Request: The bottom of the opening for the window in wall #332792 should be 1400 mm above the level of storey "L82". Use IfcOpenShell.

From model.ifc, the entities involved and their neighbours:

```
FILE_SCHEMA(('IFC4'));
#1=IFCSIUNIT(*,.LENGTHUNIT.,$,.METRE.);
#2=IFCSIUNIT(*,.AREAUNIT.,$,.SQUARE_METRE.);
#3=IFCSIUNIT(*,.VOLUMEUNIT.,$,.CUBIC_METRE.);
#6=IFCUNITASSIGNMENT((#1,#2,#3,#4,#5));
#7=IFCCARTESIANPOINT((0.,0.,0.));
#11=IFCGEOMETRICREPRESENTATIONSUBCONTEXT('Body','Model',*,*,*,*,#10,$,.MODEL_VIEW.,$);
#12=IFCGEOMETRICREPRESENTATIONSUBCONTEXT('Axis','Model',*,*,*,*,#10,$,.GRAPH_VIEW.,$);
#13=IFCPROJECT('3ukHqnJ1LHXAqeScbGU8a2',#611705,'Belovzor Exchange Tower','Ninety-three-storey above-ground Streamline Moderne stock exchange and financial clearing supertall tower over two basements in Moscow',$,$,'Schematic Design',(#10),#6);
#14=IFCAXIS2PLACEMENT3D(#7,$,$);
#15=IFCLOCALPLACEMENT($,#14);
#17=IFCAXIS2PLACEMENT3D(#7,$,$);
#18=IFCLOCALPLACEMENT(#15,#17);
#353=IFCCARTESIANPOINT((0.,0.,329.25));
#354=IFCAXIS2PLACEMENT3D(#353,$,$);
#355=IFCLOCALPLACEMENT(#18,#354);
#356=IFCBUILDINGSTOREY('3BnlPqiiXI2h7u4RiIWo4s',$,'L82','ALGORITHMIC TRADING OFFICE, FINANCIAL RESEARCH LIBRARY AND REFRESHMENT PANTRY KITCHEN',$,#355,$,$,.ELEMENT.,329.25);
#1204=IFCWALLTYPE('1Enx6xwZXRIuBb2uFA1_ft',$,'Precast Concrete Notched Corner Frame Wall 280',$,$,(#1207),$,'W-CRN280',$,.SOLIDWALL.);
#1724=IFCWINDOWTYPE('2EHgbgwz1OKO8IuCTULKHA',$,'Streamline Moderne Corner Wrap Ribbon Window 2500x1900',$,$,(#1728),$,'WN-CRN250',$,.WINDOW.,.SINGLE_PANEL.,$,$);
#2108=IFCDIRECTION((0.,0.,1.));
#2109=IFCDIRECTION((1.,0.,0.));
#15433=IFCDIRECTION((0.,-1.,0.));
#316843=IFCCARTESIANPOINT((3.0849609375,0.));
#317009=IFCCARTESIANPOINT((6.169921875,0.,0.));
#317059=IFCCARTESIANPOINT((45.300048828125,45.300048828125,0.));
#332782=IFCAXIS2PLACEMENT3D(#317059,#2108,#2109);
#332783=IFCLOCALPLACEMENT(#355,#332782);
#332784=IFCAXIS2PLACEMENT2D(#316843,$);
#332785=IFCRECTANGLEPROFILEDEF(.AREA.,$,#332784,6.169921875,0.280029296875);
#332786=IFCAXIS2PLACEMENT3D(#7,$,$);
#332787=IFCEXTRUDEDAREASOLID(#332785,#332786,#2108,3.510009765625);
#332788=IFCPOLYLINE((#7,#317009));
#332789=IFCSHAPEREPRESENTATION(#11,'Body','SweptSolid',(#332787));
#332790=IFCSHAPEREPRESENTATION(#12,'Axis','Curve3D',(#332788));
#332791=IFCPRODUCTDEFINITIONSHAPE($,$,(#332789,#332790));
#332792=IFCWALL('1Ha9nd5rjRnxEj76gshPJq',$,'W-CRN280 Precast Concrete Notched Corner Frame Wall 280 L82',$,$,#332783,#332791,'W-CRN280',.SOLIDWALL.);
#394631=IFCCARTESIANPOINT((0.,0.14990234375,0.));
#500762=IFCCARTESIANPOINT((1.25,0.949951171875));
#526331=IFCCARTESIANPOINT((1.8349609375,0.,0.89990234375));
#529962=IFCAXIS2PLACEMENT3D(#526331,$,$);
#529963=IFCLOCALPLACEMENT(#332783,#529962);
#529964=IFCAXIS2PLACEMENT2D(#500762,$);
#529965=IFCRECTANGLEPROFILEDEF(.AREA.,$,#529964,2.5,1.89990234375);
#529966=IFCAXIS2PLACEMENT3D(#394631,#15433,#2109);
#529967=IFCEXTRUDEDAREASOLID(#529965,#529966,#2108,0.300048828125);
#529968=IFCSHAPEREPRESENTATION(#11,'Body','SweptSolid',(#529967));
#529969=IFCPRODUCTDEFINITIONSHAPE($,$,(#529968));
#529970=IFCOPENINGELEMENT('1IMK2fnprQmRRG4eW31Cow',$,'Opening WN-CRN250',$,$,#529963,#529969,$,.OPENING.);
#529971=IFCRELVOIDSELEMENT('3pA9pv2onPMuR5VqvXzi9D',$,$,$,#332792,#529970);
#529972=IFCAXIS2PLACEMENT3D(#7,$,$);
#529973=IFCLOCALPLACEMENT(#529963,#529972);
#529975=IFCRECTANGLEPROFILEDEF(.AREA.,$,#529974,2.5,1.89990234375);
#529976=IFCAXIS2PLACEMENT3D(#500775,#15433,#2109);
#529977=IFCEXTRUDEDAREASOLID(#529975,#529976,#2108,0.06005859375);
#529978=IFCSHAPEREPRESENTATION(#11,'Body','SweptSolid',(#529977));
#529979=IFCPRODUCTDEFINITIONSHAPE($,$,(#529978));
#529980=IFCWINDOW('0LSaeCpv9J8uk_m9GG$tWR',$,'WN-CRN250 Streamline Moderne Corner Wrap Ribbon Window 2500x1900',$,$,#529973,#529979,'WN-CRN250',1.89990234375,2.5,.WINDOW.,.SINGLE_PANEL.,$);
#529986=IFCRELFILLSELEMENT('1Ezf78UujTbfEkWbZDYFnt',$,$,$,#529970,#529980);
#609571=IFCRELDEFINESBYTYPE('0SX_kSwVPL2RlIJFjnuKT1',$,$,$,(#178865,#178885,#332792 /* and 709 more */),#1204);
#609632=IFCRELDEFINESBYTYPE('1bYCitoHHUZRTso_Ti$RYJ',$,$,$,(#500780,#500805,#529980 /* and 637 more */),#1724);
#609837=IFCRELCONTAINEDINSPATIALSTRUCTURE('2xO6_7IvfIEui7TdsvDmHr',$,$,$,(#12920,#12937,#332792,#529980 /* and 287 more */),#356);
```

```python
import numpy as np
import ifcopenshell
import ifcopenshell.api.geometry
import ifcopenshell.geom
import ifcopenshell.util.element
import ifcopenshell.util.placement
import ifcopenshell.util.shape
import ifcopenshell.util.unit

model = ifcopenshell.open("model.ifc")
unit_scale = ifcopenshell.util.unit.calculate_unit_scale(model)

window = model.by_guid("0LSaeCpv9J8uk_m9GG$tWR")
opening = window.FillsVoids[0].RelatingOpeningElement
storey = ifcopenshell.util.element.get_container(window, ifc_class="IfcBuildingStorey")
level = ifcopenshell.util.placement.get_local_placement(storey.ObjectPlacement)[2, 3]

# The opening's origin need not be at the sill, so measure its lowest point.
shape = ifcopenshell.geom.create_shape(ifcopenshell.geom.settings(), opening)
bottom = ifcopenshell.util.shape.get_shape_bottom_elevation(shape, shape.geometry) / unit_scale
dz = level + 1.4 / unit_scale - bottom

shift = np.array([0.0, 0.0, dz])
# The window is placed relative to its opening, so it follows when the opening moves.
matrix = ifcopenshell.util.placement.get_local_placement(opening.ObjectPlacement)
matrix[:3, 3] += shift
ifcopenshell.api.geometry.edit_object_placement(
    model, product=opening, matrix=matrix, is_si=False, should_transform_children=True
)

print(f"moved by {dz * unit_scale:+.3f} m")

model.write("model_edited.ifc")
```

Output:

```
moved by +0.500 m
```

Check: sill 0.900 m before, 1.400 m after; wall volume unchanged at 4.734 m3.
